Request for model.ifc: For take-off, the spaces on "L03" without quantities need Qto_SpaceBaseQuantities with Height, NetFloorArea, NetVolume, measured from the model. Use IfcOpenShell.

First a look at what the model holds.

```python
import ifcopenshell
import ifcopenshell.util.element
import ifcopenshell.util.unit

model = ifcopenshell.open("model.ifc")
print(model.schema)
for unit_type in ("LENGTHUNIT", "AREAUNIT", "VOLUMEUNIT"):
    print(unit_type, ifcopenshell.util.unit.calculate_unit_scale(model, unit_type))
storey = next(s for s in model.by_type("IfcBuildingStorey") if s.Name == "L03")
spaces = [e for e in ifcopenshell.util.element.get_decomposition(storey) if e.is_a("IfcSpace")]
for e in sorted(spaces, key=lambda e: e.id()):
    print(e.id(), e.is_a(), e.Name, list(ifcopenshell.util.element.get_psets(e, qtos_only=True)), sep=" | ")
```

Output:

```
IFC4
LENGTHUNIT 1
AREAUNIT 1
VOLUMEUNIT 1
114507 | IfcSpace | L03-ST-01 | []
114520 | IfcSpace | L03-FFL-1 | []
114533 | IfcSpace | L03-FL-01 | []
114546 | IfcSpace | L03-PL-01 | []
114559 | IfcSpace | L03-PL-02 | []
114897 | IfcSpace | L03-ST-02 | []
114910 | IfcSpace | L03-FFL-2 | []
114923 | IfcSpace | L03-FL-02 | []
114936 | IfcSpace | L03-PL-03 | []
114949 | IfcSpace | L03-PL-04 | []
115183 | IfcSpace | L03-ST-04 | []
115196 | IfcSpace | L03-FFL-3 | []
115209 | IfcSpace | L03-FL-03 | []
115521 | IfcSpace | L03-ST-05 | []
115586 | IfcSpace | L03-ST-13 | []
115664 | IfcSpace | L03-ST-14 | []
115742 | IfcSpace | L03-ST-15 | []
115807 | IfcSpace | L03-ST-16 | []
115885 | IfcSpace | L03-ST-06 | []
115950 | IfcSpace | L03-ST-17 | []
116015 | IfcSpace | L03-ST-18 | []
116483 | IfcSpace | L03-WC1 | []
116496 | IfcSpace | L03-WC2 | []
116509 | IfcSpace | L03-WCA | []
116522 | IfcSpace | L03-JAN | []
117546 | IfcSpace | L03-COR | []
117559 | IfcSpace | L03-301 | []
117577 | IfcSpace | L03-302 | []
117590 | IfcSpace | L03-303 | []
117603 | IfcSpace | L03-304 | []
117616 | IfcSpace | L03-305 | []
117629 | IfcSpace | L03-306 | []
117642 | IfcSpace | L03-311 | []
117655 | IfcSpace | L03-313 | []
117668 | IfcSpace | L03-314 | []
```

```python
import ifcopenshell
import ifcopenshell.api.pset
import ifcopenshell.geom
import ifcopenshell.util.element
import ifcopenshell.util.shape
import ifcopenshell.util.unit

model = ifcopenshell.open("model.ifc")
unit_scale = ifcopenshell.util.unit.calculate_unit_scale(model)
area_scale = ifcopenshell.util.unit.calculate_unit_scale(model, "AREAUNIT")
volume_scale = ifcopenshell.util.unit.calculate_unit_scale(model, "VOLUMEUNIT")
settings = ifcopenshell.geom.settings()

storey = next(s for s in model.by_type("IfcBuildingStorey") if s.Name == "L03")
spaces = [e for e in ifcopenshell.util.element.get_decomposition(storey) if e.is_a("IfcSpace")]

for e in sorted(spaces, key=lambda e: e.id()):
    if ifcopenshell.util.element.get_psets(e, qtos_only=True, should_inherit=False):
        continue
    # Geometry comes back in metres, in the element's own axes.
    shape = ifcopenshell.geom.create_shape(settings, e)
    values = {
        "Height": ifcopenshell.util.shape.get_z(shape.geometry) / unit_scale,
        "NetFloorArea": ifcopenshell.util.shape.get_footprint_area(shape.geometry) / area_scale,
        "NetVolume": ifcopenshell.util.shape.get_volume(shape.geometry) / volume_scale,
    }
    qto = ifcopenshell.api.pset.add_qto(model, product=e, name="Qto_SpaceBaseQuantities")
    ifcopenshell.api.pset.edit_qto(model, qto=qto, properties=values)
    print(e.id(), {k: round(v, 3) for k, v in values.items()})

model.write("model_v2.ifc")
```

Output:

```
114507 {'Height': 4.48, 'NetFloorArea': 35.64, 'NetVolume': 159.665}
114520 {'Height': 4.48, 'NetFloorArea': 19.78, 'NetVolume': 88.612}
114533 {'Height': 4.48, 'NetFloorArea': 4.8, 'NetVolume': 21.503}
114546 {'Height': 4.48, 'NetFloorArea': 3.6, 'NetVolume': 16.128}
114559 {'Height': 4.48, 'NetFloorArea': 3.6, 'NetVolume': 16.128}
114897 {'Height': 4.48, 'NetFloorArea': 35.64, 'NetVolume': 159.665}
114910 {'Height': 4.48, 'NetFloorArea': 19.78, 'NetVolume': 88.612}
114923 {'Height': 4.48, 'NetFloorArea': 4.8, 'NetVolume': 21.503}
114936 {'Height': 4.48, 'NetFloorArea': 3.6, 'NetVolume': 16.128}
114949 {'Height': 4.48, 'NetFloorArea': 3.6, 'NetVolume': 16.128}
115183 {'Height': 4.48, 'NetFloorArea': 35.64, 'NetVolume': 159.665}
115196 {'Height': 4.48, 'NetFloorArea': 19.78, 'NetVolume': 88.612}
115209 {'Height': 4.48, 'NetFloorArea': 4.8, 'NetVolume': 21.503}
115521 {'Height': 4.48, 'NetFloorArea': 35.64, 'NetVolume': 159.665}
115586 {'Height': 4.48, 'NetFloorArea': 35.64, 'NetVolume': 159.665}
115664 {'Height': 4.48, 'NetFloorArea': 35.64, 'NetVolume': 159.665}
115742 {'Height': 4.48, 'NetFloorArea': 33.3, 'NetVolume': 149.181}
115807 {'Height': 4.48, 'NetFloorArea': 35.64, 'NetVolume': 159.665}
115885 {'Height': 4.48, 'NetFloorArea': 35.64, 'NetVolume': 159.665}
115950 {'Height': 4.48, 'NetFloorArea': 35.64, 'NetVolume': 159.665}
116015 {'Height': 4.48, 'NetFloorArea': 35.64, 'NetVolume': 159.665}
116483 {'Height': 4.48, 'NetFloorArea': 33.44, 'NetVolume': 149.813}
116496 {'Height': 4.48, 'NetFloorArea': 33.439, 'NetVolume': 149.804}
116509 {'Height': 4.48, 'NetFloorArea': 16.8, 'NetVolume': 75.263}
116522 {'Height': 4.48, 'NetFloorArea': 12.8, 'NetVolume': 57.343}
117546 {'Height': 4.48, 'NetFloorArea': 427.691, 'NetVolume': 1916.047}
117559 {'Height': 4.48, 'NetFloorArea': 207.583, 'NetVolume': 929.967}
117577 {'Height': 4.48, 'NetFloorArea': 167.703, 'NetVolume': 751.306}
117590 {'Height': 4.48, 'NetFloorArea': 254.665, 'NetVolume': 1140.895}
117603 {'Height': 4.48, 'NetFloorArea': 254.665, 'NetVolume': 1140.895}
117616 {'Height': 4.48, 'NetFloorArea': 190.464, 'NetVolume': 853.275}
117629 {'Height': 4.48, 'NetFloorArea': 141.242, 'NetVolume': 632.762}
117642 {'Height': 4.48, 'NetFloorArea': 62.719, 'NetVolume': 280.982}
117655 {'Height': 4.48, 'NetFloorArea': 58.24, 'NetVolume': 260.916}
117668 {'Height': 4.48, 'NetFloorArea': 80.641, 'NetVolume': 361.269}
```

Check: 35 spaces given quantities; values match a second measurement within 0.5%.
